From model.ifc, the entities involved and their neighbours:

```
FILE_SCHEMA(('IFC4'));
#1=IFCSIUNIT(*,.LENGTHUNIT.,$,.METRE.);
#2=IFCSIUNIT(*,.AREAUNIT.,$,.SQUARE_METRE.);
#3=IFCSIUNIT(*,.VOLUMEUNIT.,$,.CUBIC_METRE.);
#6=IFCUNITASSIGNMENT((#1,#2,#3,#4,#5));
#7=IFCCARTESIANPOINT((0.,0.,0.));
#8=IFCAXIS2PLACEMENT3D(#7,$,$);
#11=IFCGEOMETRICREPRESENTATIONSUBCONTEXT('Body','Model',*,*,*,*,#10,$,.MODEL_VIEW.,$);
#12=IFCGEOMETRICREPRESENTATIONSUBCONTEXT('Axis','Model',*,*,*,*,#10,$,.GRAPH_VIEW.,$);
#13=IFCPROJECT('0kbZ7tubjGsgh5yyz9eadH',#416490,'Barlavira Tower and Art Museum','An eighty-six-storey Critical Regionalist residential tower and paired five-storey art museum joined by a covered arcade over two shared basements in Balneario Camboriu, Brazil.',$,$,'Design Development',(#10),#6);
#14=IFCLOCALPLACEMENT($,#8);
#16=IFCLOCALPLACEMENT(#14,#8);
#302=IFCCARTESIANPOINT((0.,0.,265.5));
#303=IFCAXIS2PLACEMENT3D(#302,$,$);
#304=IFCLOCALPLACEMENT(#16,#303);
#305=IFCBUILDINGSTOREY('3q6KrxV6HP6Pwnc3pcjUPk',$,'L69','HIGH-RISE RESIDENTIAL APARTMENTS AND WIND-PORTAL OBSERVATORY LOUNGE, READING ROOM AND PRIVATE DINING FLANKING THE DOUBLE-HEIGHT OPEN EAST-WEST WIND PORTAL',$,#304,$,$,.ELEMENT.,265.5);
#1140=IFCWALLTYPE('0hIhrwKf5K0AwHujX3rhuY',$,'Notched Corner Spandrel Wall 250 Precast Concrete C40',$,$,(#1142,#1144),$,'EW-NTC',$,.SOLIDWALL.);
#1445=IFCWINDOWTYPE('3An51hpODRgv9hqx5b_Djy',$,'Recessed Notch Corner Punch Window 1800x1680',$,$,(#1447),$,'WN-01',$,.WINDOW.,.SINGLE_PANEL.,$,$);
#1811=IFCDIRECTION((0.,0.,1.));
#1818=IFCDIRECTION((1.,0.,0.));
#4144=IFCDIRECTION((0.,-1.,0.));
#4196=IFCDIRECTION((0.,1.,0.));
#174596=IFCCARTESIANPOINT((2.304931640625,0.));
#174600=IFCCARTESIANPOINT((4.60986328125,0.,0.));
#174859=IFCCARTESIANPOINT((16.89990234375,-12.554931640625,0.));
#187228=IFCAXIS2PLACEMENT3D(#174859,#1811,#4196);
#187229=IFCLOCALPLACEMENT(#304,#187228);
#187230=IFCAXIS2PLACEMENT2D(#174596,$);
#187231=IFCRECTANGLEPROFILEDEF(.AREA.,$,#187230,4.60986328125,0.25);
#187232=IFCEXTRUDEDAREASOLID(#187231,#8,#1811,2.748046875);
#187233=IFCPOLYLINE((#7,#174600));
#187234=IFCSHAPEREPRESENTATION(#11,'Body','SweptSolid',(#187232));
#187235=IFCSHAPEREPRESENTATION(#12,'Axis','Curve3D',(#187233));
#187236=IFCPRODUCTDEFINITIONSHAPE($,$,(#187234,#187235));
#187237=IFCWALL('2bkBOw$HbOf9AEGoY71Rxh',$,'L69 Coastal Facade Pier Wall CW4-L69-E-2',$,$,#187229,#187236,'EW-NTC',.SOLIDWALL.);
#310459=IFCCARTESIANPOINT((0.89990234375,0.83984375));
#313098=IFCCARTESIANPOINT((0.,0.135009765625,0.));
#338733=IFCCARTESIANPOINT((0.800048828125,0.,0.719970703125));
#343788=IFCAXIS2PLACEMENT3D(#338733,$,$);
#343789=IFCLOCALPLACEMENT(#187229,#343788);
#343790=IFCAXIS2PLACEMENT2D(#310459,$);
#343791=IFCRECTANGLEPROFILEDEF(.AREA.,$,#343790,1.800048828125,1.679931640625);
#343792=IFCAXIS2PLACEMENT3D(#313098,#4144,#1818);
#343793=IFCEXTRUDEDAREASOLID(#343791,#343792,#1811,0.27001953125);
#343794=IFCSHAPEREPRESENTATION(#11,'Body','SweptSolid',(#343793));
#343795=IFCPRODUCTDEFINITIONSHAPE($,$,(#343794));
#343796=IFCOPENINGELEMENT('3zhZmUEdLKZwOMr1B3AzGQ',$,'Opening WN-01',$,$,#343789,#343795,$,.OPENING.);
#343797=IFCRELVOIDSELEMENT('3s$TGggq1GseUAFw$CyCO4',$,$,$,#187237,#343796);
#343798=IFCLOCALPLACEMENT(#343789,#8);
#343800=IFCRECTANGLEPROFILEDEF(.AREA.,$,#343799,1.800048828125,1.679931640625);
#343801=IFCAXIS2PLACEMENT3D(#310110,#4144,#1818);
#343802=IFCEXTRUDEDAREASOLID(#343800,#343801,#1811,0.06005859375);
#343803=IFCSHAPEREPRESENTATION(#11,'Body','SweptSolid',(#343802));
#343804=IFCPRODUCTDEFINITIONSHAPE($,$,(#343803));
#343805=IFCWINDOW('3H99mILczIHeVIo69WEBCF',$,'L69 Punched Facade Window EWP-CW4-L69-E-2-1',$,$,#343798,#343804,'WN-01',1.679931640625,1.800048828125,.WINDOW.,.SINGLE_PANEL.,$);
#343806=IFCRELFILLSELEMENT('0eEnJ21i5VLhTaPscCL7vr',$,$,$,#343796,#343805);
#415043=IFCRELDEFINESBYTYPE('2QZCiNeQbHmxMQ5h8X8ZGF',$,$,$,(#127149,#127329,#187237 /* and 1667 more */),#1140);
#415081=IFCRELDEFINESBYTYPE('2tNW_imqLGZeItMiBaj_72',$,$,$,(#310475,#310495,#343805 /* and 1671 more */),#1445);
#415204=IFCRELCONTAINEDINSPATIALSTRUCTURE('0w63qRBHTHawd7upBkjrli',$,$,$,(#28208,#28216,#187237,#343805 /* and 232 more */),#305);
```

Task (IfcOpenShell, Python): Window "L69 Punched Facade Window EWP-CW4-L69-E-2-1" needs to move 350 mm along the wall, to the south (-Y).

```python
import ifcopenshell
import ifcopenshell.api.geometry
import ifcopenshell.util.placement

model = ifcopenshell.open("model.ifc")

window = model.by_id(343805)
opening = window.FillsVoids[0].RelatingOpeningElement
wall = opening.VoidsElements[0].RelatingBuildingElement

wall_matrix = ifcopenshell.util.placement.get_local_placement(wall.ObjectPlacement)
shift = wall_matrix[:3, 0] * -0.35
before = ifcopenshell.util.placement.get_local_placement(window.ObjectPlacement)[:3, 3].copy()

# The window is placed relative to its opening, so it follows when the opening moves.
matrix = ifcopenshell.util.placement.get_local_placement(opening.ObjectPlacement)
matrix[:3, 3] += shift
ifcopenshell.api.geometry.edit_object_placement(
    model, product=opening, matrix=matrix, is_si=False, should_transform_children=True
)

after = ifcopenshell.util.placement.get_local_placement(window.ObjectPlacement)[:3, 3]
print("window moved by", (after - before).round(3) + 0.0)

model.write("model-out.ifc")
```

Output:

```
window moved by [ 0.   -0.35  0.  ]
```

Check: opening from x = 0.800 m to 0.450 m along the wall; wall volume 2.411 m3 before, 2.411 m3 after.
